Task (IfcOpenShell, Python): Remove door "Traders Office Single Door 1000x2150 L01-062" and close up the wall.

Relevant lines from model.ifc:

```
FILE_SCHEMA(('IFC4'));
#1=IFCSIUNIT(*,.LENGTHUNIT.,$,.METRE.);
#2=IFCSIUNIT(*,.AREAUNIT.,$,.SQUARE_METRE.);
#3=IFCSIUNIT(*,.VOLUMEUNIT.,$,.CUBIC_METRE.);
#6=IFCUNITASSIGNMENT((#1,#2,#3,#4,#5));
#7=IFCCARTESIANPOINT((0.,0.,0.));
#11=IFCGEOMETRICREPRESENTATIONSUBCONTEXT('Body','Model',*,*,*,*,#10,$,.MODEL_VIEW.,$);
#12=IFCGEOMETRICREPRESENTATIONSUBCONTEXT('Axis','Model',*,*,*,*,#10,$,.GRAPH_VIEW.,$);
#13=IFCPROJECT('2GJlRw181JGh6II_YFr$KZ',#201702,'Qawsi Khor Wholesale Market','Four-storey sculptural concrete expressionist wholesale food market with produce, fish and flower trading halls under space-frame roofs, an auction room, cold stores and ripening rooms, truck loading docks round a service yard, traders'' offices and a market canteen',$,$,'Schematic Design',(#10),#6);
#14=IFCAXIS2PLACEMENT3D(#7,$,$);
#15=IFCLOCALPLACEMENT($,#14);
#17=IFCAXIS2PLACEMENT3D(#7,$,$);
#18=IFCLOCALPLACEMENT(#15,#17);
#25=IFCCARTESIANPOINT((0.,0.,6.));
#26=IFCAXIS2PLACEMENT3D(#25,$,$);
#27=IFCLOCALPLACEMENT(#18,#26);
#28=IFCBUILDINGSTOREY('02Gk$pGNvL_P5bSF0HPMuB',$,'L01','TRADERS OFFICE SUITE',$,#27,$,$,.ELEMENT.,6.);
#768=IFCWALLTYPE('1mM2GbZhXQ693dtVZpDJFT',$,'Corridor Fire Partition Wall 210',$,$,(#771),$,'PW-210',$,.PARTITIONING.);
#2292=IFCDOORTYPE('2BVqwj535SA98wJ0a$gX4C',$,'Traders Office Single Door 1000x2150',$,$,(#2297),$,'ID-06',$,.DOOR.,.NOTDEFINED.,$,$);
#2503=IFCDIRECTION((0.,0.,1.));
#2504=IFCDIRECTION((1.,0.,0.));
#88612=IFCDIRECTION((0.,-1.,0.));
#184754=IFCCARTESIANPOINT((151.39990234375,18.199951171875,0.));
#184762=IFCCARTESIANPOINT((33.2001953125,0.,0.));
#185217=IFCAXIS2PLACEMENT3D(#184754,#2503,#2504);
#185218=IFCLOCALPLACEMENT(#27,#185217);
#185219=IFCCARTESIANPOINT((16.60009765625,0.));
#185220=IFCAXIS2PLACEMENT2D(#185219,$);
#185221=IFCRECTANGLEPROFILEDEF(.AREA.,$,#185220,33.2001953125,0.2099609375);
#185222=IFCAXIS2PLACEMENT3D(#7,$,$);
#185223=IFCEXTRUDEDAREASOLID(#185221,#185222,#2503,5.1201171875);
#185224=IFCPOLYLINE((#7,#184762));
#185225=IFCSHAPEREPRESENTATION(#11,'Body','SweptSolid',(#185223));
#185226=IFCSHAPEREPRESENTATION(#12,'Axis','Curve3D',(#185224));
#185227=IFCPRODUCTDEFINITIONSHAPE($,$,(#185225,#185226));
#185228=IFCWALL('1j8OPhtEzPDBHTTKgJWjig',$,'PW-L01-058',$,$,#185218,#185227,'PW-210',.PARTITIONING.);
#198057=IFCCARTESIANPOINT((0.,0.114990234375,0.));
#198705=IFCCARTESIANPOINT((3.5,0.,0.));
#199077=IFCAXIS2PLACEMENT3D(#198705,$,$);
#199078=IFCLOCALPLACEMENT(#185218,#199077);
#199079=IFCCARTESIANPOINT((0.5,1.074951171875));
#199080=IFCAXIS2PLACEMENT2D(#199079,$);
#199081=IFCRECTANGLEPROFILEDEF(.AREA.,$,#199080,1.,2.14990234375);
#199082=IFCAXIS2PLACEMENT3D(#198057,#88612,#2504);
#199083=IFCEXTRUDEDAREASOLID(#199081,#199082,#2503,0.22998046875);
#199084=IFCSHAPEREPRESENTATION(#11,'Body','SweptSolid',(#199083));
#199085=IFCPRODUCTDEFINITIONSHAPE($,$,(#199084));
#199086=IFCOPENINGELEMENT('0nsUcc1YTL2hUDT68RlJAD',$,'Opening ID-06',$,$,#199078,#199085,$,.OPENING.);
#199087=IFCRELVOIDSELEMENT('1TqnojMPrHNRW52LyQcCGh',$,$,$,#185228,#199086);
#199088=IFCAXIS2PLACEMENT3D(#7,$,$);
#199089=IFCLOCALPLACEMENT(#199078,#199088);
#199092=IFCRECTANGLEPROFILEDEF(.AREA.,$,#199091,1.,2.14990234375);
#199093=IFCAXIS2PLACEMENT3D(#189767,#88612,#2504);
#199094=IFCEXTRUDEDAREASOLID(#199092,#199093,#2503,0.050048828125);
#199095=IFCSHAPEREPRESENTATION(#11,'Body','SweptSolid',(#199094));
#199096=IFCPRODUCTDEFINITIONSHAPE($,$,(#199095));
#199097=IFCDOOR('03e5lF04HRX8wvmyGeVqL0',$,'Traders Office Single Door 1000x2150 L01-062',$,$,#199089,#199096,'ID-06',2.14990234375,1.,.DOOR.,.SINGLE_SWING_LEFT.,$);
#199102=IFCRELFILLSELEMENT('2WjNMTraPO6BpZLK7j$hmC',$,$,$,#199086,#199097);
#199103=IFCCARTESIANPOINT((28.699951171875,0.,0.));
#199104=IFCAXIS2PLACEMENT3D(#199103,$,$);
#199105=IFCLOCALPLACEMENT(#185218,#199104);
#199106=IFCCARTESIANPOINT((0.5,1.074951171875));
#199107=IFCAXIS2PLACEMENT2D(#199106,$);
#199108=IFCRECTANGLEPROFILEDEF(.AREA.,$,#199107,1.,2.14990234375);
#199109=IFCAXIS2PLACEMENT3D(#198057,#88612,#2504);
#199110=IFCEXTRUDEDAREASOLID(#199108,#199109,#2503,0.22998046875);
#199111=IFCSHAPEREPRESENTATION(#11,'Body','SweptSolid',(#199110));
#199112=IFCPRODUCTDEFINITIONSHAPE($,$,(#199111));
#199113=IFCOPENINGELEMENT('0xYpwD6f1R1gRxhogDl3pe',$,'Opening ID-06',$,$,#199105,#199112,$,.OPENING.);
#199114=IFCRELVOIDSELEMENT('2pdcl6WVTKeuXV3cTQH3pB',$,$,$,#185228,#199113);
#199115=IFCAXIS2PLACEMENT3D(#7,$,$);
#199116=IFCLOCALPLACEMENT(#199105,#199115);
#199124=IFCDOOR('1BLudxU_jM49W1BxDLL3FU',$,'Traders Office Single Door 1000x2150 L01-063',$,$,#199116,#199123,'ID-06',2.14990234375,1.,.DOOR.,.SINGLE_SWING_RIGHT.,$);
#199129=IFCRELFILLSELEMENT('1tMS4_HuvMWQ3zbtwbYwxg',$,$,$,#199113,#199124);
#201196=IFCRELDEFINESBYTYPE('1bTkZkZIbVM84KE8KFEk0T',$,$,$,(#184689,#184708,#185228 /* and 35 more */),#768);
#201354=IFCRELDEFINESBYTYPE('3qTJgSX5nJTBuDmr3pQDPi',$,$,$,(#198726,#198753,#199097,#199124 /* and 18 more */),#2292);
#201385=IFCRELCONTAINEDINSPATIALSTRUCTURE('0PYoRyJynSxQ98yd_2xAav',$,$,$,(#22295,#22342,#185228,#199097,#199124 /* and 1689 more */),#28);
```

```python
import ifcopenshell
import ifcopenshell.api.feature
import ifcopenshell.api.root
import ifcopenshell.geom
import ifcopenshell.util.shape

model = ifcopenshell.open("model.ifc")
settings = ifcopenshell.geom.settings()


def volume(element):
    """Net volume in cubic metres, openings subtracted."""
    shape = ifcopenshell.geom.create_shape(settings, element)
    return ifcopenshell.util.shape.get_volume(shape.geometry)


door = model.by_guid("03e5lF04HRX8wvmyGeVqL0")
opening = door.FillsVoids[0].RelatingOpeningElement
wall = opening.VoidsElements[0].RelatingBuildingElement
before = volume(wall)

ifcopenshell.api.root.remove_product(model, product=door)
ifcopenshell.api.feature.remove_feature(model, feature=opening)

after = volume(wall)

print(f"wall volume {before:.3f} -> {after:.3f} m3")

model.write("model_edited.ifc")
```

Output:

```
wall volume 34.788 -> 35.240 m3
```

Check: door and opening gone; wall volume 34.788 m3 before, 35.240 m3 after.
